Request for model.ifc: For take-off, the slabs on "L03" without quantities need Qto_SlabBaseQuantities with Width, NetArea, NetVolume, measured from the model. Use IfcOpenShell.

First a look at what the model holds.

```python
import ifcopenshell
import ifcopenshell.util.element
import ifcopenshell.util.unit

model = ifcopenshell.open("model.ifc")
print(model.schema)
for unit_type in ("LENGTHUNIT", "AREAUNIT", "VOLUMEUNIT"):
    print(unit_type, ifcopenshell.util.unit.calculate_unit_scale(model, unit_type))
storey = next(s for s in model.by_type("IfcBuildingStorey") if s.Name == "L03")
slabs = [e for e in ifcopenshell.util.element.get_decomposition(storey) if e.is_a("IfcSlab")]
for e in sorted(slabs, key=lambda e: e.id()):
    print(e.id(), e.is_a(), e.Name, list(ifcopenshell.util.element.get_psets(e, qtos_only=True)), sep=" | ")
```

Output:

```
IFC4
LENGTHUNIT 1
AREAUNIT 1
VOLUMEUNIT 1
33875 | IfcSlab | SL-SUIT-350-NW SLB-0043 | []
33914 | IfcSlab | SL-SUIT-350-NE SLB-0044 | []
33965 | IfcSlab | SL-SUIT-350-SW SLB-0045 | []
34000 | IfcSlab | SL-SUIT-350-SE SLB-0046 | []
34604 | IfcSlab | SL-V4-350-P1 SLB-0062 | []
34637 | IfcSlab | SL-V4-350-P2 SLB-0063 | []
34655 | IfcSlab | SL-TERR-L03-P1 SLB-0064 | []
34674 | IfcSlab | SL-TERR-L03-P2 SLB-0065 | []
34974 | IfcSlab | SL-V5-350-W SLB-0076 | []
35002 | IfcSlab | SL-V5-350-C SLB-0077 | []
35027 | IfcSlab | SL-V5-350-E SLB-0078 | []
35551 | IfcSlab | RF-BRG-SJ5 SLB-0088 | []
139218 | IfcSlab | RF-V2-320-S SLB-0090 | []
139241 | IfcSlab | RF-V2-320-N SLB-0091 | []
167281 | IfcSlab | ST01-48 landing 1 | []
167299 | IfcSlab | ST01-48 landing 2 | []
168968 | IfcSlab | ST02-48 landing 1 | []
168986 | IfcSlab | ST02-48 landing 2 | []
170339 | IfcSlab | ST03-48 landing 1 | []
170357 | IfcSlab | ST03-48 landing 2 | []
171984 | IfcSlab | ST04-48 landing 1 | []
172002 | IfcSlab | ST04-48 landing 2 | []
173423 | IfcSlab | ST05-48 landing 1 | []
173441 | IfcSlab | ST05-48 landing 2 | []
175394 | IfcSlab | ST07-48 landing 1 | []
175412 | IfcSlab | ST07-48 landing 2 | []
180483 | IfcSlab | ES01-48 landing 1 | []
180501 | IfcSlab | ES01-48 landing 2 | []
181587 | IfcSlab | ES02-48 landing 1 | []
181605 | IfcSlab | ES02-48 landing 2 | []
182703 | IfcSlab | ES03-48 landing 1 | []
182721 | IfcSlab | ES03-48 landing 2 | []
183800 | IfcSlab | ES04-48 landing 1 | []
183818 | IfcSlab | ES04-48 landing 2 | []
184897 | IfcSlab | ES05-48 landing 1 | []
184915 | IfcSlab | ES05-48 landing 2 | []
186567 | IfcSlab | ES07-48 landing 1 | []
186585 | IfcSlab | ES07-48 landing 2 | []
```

```python
import ifcopenshell
import ifcopenshell.api.pset
import ifcopenshell.geom
import ifcopenshell.util.element
import ifcopenshell.util.shape
import ifcopenshell.util.unit

model = ifcopenshell.open("model.ifc")
unit_scale = ifcopenshell.util.unit.calculate_unit_scale(model)
area_scale = ifcopenshell.util.unit.calculate_unit_scale(model, "AREAUNIT")
volume_scale = ifcopenshell.util.unit.calculate_unit_scale(model, "VOLUMEUNIT")
settings = ifcopenshell.geom.settings()

storey = next(s for s in model.by_type("IfcBuildingStorey") if s.Name == "L03")
slabs = [e for e in ifcopenshell.util.element.get_decomposition(storey) if e.is_a("IfcSlab")]

for e in sorted(slabs, key=lambda e: e.id()):
    if ifcopenshell.util.element.get_psets(e, qtos_only=True, should_inherit=False):
        continue
    # Geometry comes back in metres, in the element's own axes.
    shape = ifcopenshell.geom.create_shape(settings, e)
    values = {
        "Width": ifcopenshell.util.shape.get_z(shape.geometry) / unit_scale,
        "NetArea": ifcopenshell.util.shape.get_footprint_area(shape.geometry) / area_scale,
        "NetVolume": ifcopenshell.util.shape.get_volume(shape.geometry) / volume_scale,
    }
    qto = ifcopenshell.api.pset.add_qto(model, product=e, name="Qto_SlabBaseQuantities")
    ifcopenshell.api.pset.edit_qto(model, qto=qto, properties=values)
    print(e.id(), {k: round(v, 3) for k, v in values.items()})

model.write("model_v2.ifc")
```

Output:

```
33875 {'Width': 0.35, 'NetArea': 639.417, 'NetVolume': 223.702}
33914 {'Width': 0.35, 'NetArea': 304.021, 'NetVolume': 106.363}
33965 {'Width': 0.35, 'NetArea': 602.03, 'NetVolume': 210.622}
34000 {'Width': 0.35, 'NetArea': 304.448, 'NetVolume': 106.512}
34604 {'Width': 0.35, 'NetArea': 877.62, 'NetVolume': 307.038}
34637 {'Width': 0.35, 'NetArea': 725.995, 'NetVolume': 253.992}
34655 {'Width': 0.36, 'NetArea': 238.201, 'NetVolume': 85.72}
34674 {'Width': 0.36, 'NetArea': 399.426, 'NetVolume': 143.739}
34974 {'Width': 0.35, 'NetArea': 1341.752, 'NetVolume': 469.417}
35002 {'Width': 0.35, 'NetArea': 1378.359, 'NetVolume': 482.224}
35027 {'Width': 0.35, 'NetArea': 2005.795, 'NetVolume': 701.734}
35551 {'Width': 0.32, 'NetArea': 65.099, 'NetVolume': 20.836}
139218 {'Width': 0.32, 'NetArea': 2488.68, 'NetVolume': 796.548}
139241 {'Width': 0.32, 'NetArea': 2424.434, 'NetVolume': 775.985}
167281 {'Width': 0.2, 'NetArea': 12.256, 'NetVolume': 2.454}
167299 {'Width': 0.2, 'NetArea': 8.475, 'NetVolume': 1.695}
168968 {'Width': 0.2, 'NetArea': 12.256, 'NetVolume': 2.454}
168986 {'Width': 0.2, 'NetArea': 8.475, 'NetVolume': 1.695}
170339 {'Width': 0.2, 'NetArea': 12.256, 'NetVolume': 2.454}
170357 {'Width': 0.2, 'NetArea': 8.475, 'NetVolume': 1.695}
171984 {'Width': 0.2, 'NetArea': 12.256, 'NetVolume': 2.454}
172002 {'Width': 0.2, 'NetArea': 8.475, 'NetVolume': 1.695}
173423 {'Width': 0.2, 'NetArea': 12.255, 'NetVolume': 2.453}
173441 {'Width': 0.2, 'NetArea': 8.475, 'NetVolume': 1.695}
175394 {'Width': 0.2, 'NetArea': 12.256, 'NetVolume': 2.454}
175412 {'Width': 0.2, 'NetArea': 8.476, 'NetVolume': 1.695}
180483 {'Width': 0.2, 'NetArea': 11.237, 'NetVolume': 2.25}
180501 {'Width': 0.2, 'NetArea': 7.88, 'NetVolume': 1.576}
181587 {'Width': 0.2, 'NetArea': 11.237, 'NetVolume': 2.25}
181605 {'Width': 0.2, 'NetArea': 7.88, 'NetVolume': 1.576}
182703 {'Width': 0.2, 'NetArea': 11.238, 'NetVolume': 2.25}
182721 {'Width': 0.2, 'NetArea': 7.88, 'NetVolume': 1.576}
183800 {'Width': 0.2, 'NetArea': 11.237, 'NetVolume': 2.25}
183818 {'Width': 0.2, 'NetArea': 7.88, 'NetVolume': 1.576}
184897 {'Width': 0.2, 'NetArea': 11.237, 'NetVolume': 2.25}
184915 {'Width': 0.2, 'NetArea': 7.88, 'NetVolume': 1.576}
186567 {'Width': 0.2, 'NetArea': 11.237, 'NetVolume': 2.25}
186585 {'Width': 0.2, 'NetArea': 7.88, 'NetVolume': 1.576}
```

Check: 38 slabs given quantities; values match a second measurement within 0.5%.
